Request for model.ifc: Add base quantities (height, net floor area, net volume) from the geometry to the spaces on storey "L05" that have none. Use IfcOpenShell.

First a look at what the model holds.

```python
import ifcopenshell
import ifcopenshell.util.element
import ifcopenshell.util.unit

model = ifcopenshell.open("model.ifc")
print(model.schema)
for unit_type in ("LENGTHUNIT", "AREAUNIT", "VOLUMEUNIT"):
    print(unit_type, ifcopenshell.util.unit.calculate_unit_scale(model, unit_type))
storey = next(s for s in model.by_type("IfcBuildingStorey") if s.Name == "L05")
spaces = [e for e in ifcopenshell.util.element.get_decomposition(storey) if e.is_a("IfcSpace")]
for e in sorted(spaces, key=lambda e: e.id()):
    print(e.id(), e.is_a(), e.Name, list(ifcopenshell.util.element.get_psets(e, qtos_only=True)), sep=" | ")
```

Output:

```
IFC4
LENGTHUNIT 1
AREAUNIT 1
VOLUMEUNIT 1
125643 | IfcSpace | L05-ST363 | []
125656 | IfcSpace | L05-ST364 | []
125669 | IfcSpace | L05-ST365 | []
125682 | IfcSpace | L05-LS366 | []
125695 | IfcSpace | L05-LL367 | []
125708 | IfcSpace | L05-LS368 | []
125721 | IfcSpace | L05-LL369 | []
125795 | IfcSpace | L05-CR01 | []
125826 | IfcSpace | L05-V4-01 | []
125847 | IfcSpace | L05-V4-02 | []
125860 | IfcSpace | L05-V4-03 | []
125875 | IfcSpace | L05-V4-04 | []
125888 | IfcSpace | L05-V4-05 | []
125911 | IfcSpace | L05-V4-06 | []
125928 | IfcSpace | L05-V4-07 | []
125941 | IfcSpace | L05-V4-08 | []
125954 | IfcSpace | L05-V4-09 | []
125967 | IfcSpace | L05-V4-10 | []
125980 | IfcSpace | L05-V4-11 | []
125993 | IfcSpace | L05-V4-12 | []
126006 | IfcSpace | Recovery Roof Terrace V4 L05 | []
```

```python
import ifcopenshell
import ifcopenshell.api.pset
import ifcopenshell.geom
import ifcopenshell.util.element
import ifcopenshell.util.shape
import ifcopenshell.util.unit

model = ifcopenshell.open("model.ifc")
unit_scale = ifcopenshell.util.unit.calculate_unit_scale(model)
area_scale = ifcopenshell.util.unit.calculate_unit_scale(model, "AREAUNIT")
volume_scale = ifcopenshell.util.unit.calculate_unit_scale(model, "VOLUMEUNIT")
settings = ifcopenshell.geom.settings()

storey = next(s for s in model.by_type("IfcBuildingStorey") if s.Name == "L05")
spaces = [e for e in ifcopenshell.util.element.get_decomposition(storey) if e.is_a("IfcSpace")]

for e in sorted(spaces, key=lambda e: e.id()):
    if ifcopenshell.util.element.get_psets(e, qtos_only=True, should_inherit=False):
        continue
    # Geometry comes back in metres, in the element's own axes.
    shape = ifcopenshell.geom.create_shape(settings, e)
    values = {
        "Height": ifcopenshell.util.shape.get_z(shape.geometry) / unit_scale,
        "NetFloorArea": ifcopenshell.util.shape.get_footprint_area(shape.geometry) / area_scale,
        "NetVolume": ifcopenshell.util.shape.get_volume(shape.geometry) / volume_scale,
    }
    qto = ifcopenshell.api.pset.add_qto(model, product=e, name="Qto_SpaceBaseQuantities")
    ifcopenshell.api.pset.edit_qto(model, qto=qto, properties=values)
    print(e.id(), {k: round(v, 3) for k, v in values.items()})

model.write("model_updated.ifc")
```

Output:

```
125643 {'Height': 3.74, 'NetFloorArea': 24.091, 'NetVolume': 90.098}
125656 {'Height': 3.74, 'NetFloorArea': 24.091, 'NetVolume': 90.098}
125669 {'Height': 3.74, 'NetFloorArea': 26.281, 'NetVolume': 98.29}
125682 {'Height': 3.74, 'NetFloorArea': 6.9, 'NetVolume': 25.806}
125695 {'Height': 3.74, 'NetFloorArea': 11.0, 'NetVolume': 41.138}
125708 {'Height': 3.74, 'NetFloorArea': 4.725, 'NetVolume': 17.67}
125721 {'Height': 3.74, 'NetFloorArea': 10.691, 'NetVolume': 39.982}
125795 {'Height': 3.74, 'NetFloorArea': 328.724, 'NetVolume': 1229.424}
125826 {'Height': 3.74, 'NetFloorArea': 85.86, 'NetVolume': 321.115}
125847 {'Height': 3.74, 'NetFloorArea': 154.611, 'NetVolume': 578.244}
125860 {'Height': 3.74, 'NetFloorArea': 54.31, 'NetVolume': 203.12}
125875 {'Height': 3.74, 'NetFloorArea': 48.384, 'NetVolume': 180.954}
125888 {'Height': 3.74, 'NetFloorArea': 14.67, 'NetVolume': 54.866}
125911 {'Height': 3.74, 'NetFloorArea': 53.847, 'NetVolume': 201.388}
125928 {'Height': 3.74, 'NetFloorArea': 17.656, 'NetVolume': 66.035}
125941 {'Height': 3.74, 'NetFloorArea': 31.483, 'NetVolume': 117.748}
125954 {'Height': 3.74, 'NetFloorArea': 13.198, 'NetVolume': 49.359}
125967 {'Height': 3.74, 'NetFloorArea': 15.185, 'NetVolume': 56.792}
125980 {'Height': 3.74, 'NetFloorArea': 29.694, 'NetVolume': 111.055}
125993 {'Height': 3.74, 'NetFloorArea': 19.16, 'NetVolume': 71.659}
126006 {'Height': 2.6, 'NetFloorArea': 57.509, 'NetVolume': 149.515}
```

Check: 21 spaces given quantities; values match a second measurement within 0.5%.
